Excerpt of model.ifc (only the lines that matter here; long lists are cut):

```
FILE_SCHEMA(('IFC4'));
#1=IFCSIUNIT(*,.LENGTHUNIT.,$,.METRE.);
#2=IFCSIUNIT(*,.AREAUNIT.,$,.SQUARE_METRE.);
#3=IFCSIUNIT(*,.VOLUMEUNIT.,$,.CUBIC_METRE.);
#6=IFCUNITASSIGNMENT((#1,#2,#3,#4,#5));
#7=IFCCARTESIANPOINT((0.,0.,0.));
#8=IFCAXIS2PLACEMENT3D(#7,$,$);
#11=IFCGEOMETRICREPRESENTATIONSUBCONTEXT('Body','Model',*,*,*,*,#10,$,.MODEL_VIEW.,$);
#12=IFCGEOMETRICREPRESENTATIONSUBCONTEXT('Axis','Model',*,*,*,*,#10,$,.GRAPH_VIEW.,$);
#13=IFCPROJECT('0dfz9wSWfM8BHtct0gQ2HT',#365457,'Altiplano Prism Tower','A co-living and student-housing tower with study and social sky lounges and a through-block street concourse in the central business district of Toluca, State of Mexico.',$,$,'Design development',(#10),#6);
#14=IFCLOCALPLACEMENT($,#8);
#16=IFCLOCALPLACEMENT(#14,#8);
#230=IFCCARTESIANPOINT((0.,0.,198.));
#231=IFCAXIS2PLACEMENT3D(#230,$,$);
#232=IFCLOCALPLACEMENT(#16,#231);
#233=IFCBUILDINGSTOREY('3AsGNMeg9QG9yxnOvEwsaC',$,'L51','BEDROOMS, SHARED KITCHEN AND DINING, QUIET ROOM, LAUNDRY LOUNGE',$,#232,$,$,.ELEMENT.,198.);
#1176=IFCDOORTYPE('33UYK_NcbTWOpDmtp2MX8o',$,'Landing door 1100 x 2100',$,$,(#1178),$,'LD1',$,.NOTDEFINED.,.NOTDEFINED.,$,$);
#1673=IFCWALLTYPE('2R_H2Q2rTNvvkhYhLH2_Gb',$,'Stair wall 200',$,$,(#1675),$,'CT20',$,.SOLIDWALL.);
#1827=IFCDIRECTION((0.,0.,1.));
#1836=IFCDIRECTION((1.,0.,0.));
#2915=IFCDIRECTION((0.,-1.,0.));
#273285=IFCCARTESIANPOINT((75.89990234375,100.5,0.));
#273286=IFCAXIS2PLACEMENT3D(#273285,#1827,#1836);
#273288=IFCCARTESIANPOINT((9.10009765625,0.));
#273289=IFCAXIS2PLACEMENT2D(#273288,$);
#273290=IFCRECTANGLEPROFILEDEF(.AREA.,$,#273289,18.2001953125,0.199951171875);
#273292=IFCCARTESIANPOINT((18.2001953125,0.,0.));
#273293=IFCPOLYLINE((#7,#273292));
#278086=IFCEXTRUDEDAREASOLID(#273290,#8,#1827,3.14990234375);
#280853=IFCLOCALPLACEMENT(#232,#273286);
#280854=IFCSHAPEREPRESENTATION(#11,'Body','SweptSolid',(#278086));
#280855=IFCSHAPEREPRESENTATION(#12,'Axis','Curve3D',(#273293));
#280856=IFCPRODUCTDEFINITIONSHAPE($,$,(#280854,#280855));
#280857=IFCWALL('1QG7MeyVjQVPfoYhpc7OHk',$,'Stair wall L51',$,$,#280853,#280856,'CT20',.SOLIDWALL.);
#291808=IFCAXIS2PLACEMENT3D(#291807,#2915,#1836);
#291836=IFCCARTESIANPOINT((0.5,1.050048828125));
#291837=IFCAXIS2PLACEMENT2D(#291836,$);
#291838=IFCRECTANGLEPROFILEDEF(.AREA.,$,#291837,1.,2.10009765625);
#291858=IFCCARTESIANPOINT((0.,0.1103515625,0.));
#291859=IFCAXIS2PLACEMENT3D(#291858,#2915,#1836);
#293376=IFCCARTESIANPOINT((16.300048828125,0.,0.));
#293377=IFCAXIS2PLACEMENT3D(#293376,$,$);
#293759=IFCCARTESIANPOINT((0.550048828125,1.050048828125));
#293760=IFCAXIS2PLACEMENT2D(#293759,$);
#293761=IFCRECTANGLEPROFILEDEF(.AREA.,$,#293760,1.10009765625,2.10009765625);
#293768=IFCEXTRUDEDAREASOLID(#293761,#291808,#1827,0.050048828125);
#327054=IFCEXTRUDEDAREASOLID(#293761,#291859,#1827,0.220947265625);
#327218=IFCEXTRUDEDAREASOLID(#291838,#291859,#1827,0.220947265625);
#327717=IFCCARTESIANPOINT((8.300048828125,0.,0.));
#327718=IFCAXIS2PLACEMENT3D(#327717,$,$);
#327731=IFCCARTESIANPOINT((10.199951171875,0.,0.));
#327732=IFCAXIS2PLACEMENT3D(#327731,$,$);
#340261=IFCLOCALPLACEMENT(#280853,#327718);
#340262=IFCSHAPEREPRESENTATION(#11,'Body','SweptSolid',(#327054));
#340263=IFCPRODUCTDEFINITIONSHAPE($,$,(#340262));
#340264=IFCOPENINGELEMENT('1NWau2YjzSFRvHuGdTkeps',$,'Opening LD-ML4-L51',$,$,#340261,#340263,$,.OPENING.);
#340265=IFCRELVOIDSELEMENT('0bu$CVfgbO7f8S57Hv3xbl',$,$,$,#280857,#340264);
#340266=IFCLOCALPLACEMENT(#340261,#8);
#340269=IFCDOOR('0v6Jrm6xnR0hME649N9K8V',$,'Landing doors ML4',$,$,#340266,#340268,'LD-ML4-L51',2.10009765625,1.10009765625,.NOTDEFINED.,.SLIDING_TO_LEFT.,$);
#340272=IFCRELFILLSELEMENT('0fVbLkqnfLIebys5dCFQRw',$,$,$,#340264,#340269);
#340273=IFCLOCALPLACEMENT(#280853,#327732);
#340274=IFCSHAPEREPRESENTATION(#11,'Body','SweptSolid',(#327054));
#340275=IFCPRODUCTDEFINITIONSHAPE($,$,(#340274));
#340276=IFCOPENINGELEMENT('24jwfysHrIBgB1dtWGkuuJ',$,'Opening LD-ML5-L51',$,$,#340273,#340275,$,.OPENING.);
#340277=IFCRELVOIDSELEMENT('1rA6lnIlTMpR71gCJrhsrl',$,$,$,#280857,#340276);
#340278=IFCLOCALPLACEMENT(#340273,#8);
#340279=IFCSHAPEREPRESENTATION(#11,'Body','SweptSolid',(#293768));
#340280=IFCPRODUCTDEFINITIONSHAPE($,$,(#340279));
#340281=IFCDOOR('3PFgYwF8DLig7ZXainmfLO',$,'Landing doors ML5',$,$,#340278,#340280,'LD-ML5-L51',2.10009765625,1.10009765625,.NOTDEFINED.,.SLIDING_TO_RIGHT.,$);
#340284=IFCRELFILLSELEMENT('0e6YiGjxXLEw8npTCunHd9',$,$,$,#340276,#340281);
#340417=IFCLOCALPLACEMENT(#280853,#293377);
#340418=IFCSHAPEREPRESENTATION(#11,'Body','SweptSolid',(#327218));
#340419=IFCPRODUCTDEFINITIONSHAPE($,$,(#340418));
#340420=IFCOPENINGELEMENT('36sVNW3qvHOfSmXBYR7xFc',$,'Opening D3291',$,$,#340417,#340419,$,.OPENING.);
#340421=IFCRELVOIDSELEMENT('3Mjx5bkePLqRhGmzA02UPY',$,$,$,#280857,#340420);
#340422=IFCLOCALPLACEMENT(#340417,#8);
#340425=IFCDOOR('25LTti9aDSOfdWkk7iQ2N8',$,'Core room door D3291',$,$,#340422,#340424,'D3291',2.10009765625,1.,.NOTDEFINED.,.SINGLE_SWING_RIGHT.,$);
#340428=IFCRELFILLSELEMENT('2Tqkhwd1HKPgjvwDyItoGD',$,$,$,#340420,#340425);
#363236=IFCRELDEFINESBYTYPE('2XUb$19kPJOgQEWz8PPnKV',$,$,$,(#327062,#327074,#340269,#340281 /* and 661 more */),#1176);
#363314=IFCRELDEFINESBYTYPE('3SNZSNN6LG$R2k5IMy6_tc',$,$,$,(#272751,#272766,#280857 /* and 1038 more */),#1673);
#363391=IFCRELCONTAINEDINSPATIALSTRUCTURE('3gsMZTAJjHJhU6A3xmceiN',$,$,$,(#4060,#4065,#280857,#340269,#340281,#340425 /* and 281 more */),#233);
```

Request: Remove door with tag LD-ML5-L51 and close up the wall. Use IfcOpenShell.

```python
import ifcopenshell
import ifcopenshell.api.feature
import ifcopenshell.api.root
import ifcopenshell.geom
import ifcopenshell.util.shape

model = ifcopenshell.open("model.ifc")
settings = ifcopenshell.geom.settings()


def volume(element):
    """Net volume in cubic metres, openings subtracted."""
    shape = ifcopenshell.geom.create_shape(settings, element)
    return ifcopenshell.util.shape.get_volume(shape.geometry)


door = model.by_guid("3PFgYwF8DLig7ZXainmfLO")
opening = door.FillsVoids[0].RelatingOpeningElement
wall = opening.VoidsElements[0].RelatingBuildingElement
before = volume(wall)

ifcopenshell.api.root.remove_product(model, product=door)
ifcopenshell.api.feature.remove_feature(model, feature=opening)

after = volume(wall)

print(f"wall volume {before:.3f} -> {after:.3f} m3")

model.write("model_rev.ifc")
```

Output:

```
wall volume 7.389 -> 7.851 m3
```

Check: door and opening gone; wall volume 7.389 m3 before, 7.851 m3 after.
